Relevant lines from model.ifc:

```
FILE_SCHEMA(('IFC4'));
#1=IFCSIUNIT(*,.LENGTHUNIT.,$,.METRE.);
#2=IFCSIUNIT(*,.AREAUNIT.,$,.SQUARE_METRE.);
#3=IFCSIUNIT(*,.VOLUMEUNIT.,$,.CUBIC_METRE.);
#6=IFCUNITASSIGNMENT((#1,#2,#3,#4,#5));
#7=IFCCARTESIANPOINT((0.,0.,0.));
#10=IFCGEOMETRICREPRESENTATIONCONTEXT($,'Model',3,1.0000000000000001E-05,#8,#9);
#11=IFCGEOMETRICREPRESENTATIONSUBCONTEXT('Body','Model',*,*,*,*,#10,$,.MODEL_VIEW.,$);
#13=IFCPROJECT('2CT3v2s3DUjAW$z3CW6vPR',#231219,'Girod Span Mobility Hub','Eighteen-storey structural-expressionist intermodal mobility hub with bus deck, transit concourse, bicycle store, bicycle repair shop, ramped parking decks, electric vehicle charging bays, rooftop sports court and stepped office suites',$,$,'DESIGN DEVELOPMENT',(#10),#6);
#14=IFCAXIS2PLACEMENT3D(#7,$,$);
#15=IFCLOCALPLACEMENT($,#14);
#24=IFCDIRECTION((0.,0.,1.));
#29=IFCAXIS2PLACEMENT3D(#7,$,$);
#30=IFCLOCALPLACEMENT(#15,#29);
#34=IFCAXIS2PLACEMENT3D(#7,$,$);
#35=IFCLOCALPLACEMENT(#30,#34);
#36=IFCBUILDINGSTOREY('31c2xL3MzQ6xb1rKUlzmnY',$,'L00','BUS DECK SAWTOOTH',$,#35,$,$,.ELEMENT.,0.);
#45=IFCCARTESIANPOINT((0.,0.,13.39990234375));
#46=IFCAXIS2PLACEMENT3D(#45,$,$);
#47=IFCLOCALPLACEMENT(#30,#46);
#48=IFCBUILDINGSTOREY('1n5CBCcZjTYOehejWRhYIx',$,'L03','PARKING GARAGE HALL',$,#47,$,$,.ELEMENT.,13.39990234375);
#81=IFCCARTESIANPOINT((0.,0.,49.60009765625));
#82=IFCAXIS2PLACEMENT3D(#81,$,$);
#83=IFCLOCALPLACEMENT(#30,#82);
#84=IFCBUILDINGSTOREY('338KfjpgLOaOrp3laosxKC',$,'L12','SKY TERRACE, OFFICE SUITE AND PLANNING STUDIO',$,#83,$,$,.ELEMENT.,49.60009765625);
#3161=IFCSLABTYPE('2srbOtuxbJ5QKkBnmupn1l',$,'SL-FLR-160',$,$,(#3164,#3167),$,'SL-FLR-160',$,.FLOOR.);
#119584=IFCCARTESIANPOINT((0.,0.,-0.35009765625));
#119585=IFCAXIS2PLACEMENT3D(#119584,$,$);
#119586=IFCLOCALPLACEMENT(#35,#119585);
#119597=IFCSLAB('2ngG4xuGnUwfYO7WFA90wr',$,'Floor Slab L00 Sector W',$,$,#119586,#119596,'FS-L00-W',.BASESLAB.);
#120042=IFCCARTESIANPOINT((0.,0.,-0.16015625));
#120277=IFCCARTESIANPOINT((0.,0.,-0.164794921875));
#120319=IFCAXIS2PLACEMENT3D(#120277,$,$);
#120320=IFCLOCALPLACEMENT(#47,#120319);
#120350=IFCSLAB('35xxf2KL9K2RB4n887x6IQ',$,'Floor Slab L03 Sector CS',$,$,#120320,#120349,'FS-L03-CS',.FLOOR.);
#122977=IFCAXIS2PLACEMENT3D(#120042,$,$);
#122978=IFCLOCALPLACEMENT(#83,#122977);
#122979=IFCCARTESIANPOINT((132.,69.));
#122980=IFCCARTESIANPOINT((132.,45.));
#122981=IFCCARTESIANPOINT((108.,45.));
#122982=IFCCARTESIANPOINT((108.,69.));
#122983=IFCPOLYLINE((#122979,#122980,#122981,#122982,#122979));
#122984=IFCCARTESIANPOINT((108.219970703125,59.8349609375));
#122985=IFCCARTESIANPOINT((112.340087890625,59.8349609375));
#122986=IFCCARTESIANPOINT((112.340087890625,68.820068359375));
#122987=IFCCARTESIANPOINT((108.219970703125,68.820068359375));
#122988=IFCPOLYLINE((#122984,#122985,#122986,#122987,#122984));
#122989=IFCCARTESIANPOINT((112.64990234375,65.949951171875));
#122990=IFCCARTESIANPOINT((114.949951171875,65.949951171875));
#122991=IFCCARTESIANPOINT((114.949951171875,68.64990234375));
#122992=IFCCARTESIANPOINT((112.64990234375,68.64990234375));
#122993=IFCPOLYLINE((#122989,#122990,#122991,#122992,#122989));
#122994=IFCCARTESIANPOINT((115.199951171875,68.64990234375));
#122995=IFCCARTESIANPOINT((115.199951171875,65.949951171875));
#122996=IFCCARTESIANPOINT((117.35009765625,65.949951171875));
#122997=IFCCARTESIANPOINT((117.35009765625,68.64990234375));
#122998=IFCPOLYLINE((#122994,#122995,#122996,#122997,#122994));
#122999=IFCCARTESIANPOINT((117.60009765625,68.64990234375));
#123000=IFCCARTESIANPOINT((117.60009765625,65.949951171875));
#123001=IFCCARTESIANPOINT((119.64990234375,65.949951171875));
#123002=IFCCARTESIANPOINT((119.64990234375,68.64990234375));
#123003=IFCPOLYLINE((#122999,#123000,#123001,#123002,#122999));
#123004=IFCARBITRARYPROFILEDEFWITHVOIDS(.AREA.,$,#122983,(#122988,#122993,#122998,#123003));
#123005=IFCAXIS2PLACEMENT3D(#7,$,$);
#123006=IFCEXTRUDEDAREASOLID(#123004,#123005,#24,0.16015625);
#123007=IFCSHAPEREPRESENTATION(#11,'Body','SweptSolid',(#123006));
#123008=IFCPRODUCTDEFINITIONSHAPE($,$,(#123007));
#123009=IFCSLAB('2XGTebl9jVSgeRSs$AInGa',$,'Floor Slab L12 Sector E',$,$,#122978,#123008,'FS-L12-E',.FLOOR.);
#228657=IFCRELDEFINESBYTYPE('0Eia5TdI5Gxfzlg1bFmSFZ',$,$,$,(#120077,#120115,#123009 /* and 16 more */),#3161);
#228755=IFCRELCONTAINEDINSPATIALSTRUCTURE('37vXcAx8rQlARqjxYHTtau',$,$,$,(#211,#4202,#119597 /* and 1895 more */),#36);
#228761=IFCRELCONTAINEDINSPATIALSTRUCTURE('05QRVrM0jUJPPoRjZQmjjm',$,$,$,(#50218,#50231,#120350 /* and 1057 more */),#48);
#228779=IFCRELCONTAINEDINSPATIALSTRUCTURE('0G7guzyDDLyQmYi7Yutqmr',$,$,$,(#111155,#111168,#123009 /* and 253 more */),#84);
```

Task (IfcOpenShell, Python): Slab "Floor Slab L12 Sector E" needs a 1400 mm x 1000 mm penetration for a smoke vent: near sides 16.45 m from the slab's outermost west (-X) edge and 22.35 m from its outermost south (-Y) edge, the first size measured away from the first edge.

```python
import numpy as np
import ifcopenshell
import ifcopenshell.api.feature
import ifcopenshell.api.geometry
import ifcopenshell.api.root
import ifcopenshell.geom
import ifcopenshell.util.placement
import ifcopenshell.util.representation
import ifcopenshell.util.shape
import ifcopenshell.util.unit

model = ifcopenshell.open("model.ifc")
unit_scale = ifcopenshell.util.unit.calculate_unit_scale(model)
settings = ifcopenshell.geom.settings()


def volume(element):
    """Net volume in cubic metres, openings subtracted."""
    shape = ifcopenshell.geom.create_shape(settings, element)
    return ifcopenshell.util.shape.get_volume(shape.geometry)


slab = model.by_id(123009)
before = volume(slab)

# Extent in the slab's own axes, in metres. The edges named are its -X and -Y sides.
slab_shape = ifcopenshell.geom.create_shape(settings, slab)
vertices = ifcopenshell.util.shape.get_vertices(slab_shape.geometry)
x_min, y_min, bottom = vertices.min(axis=0)
top = vertices[:, 2].max()

opening = ifcopenshell.api.root.create_entity(model, ifc_class="IfcOpeningElement", name="Smoke vent opening", predefined_type="OPENING")
context = ifcopenshell.util.representation.get_context(model, "Model", "Body", "MODEL_VIEW")
width, depth = 1.4, 1
outline = [(0.0, 0.0), (width, 0.0), (width, depth), (0.0, depth), (0.0, 0.0)]
# Overshoot both faces by 50 mm so the cut is clean.
shape = ifcopenshell.api.geometry.add_slab_representation(
    model, context=context, depth=top - bottom + 0.1, polyline=outline
)
ifcopenshell.api.geometry.assign_representation(model, product=opening, representation=shape)

matrix = ifcopenshell.util.placement.get_local_placement(slab.ObjectPlacement)
matrix[:, 3] = matrix @ np.append(np.array([x_min + 16.45, y_min + 22.35, bottom - 0.05]) / unit_scale, 1.0)
ifcopenshell.api.geometry.edit_object_placement(model, product=opening, matrix=matrix, is_si=False)
ifcopenshell.api.feature.add_feature(model, feature=opening, element=slab)

after = volume(slab)

print(f"slab volume {before:.3f} -> {after:.3f} m3")

model.write("model_edited.ifc")
```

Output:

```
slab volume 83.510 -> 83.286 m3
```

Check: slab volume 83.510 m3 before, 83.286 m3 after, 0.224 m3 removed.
